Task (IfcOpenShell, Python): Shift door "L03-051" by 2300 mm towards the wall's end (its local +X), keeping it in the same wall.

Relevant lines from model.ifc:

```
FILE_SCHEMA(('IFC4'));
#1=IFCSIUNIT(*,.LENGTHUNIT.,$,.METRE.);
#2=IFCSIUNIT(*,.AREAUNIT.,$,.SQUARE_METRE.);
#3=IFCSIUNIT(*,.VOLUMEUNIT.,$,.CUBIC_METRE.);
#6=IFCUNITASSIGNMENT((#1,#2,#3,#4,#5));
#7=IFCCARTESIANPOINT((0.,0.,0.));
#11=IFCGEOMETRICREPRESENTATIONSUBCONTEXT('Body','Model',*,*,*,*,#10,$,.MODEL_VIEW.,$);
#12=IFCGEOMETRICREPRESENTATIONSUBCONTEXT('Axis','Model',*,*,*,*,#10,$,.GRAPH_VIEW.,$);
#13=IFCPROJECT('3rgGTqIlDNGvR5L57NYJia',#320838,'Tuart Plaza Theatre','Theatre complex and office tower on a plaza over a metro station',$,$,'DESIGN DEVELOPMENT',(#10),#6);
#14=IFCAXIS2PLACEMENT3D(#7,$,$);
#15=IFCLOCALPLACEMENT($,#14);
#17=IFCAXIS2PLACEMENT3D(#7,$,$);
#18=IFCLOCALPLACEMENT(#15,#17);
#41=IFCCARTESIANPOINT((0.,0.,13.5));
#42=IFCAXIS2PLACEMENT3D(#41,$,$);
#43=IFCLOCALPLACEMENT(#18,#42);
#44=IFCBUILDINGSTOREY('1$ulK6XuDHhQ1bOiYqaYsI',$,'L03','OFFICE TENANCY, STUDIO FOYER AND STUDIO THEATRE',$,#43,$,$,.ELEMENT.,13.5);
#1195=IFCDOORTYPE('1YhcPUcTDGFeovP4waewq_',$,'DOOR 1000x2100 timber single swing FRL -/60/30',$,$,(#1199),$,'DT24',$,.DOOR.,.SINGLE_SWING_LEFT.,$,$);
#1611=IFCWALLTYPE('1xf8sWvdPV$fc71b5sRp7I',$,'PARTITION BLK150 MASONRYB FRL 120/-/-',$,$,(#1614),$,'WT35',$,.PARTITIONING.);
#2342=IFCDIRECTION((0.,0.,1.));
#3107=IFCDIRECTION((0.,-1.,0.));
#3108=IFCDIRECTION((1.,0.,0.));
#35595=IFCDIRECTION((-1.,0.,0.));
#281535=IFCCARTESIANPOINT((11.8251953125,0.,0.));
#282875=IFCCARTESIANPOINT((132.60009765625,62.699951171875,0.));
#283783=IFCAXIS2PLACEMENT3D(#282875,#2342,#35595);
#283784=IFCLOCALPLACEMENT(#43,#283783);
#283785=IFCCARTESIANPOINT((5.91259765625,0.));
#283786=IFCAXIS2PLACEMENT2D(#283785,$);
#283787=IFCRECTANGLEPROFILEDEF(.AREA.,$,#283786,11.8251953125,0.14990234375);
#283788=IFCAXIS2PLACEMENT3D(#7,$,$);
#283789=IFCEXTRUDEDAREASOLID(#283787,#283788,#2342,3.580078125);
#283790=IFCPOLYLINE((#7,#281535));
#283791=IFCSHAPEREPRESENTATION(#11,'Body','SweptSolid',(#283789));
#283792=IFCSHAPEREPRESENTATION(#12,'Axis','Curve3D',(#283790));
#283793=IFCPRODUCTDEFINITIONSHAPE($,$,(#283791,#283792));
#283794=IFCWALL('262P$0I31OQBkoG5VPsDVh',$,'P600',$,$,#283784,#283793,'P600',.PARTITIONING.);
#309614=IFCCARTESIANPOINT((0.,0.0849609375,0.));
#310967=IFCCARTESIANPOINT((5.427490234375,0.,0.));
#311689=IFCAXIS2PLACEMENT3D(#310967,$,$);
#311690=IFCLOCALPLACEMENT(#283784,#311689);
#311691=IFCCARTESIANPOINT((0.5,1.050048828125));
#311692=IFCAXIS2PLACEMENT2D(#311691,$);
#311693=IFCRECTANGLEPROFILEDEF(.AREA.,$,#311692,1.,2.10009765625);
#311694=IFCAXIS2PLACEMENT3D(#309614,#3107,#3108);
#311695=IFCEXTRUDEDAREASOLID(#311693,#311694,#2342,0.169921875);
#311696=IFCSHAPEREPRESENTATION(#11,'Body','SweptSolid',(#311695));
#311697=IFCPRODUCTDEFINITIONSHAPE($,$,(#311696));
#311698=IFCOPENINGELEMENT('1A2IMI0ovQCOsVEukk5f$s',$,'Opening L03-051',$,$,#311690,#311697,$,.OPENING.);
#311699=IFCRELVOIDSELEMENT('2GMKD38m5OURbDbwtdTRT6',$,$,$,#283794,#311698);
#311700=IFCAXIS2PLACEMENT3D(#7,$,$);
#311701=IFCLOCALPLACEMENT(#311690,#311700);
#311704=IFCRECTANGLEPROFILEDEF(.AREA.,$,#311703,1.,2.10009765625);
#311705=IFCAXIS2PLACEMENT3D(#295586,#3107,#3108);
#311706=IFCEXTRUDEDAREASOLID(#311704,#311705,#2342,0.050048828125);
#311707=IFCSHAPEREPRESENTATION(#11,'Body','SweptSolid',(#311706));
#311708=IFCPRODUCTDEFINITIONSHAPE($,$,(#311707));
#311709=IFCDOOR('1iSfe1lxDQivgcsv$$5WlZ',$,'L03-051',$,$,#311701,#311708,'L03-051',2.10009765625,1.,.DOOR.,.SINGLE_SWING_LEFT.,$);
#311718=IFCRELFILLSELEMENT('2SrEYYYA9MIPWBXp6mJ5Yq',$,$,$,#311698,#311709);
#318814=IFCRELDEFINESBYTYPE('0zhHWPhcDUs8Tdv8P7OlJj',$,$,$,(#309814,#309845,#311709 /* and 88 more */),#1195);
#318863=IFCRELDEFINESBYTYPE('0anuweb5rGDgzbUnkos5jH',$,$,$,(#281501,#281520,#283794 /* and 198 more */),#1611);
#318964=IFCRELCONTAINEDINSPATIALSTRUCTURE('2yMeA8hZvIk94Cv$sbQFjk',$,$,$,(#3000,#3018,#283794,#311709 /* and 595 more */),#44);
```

```python
import ifcopenshell
import ifcopenshell.api.geometry
import ifcopenshell.util.placement
import ifcopenshell.util.unit

model = ifcopenshell.open("model.ifc")
unit_scale = ifcopenshell.util.unit.calculate_unit_scale(model)

door = model.by_guid("1iSfe1lxDQivgcsv$$5WlZ")
opening = door.FillsVoids[0].RelatingOpeningElement
wall = opening.VoidsElements[0].RelatingBuildingElement

wall_matrix = ifcopenshell.util.placement.get_local_placement(wall.ObjectPlacement)
shift = wall_matrix[:3, 0] * 2.3 / unit_scale
before = ifcopenshell.util.placement.get_local_placement(door.ObjectPlacement)[:3, 3].copy()

# The door is placed relative to its opening, so it follows when the opening moves.
matrix = ifcopenshell.util.placement.get_local_placement(opening.ObjectPlacement)
matrix[:3, 3] += shift
ifcopenshell.api.geometry.edit_object_placement(
    model, product=opening, matrix=matrix, is_si=False, should_transform_children=True
)

after = ifcopenshell.util.placement.get_local_placement(door.ObjectPlacement)[:3, 3]
print("door moved by", (after - before).round(3) + 0.0)

model.write("model_v2.ifc")
```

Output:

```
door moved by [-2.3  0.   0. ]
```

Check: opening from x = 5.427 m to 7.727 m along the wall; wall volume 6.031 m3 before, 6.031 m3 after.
